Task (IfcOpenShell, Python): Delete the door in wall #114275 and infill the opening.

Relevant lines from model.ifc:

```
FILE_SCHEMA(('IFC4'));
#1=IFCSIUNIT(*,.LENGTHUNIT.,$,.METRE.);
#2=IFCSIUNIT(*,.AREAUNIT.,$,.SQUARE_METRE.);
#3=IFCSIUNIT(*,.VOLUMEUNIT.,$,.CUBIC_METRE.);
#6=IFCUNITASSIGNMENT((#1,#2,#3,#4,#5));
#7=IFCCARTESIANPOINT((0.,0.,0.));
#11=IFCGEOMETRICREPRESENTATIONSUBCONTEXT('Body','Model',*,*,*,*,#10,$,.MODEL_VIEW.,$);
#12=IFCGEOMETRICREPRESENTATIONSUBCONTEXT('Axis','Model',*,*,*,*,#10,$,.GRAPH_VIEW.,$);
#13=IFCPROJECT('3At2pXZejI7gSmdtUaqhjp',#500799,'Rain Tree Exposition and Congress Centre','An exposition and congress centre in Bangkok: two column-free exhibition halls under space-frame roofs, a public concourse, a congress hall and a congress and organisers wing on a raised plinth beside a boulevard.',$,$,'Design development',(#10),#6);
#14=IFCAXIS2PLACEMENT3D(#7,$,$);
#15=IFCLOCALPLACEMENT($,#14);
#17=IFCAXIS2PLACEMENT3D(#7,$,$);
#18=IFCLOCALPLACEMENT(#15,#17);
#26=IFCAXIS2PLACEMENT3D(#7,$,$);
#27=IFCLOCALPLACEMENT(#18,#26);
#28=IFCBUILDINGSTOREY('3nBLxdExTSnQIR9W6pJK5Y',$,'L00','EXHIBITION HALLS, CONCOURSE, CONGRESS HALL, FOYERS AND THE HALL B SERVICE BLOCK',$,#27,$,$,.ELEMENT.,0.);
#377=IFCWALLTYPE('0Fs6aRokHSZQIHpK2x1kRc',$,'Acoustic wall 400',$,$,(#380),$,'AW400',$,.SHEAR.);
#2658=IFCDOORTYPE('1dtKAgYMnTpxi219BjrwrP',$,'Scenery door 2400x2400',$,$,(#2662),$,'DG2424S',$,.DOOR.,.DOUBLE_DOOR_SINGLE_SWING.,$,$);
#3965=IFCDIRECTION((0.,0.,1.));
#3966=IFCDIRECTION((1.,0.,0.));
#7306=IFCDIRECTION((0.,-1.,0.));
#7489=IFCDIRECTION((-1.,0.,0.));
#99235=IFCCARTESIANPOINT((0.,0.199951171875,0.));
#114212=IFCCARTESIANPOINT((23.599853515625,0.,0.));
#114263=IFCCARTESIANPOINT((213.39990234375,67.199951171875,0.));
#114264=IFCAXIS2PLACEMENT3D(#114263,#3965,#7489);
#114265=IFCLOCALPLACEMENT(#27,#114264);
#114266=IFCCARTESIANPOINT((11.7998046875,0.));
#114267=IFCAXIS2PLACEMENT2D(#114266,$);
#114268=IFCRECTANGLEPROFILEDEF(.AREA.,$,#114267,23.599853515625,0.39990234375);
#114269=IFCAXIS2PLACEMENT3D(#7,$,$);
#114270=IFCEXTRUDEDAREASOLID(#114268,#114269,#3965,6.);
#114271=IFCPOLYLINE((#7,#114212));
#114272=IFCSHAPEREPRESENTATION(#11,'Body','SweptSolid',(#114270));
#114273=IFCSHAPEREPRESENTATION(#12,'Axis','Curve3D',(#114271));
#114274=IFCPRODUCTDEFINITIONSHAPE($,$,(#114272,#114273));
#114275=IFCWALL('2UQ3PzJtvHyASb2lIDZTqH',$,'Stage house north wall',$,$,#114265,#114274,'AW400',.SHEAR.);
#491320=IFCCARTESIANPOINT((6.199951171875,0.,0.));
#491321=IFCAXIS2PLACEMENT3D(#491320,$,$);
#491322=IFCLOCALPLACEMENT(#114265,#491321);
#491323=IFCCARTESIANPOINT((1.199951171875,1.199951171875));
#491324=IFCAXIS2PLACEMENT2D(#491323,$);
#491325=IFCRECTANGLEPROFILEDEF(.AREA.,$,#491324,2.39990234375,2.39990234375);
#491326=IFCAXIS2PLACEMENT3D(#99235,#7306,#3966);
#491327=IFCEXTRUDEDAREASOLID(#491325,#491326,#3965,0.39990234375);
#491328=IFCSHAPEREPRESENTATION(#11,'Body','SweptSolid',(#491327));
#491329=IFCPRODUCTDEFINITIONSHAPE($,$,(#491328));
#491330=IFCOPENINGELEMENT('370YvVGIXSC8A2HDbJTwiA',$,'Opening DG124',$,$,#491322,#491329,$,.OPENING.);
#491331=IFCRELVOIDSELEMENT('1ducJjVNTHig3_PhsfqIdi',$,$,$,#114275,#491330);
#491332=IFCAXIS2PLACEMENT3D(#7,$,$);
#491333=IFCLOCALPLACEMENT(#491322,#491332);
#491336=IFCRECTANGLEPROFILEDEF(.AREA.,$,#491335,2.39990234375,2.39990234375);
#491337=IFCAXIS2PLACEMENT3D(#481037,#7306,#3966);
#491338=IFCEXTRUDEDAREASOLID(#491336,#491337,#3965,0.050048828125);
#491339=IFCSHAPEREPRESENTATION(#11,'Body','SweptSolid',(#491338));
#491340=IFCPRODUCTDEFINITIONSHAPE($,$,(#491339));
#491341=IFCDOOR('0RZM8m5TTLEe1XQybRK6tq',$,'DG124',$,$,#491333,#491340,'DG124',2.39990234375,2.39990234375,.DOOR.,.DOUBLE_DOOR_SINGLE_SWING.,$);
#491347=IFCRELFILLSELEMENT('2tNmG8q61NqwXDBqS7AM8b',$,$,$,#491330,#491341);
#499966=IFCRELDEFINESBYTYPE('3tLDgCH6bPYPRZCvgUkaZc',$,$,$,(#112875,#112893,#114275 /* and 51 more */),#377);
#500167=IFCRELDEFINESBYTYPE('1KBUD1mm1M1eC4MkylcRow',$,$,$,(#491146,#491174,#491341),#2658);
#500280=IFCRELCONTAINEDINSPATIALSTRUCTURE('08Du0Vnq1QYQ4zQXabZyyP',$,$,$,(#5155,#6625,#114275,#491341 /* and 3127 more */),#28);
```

```python
import ifcopenshell
import ifcopenshell.api.feature
import ifcopenshell.api.root
import ifcopenshell.geom
import ifcopenshell.util.shape

model = ifcopenshell.open("model.ifc")
settings = ifcopenshell.geom.settings()


def volume(element):
    """Net volume in cubic metres, openings subtracted."""
    shape = ifcopenshell.geom.create_shape(settings, element)
    return ifcopenshell.util.shape.get_volume(shape.geometry)


door = model.by_guid("0RZM8m5TTLEe1XQybRK6tq")
opening = door.FillsVoids[0].RelatingOpeningElement
wall = opening.VoidsElements[0].RelatingBuildingElement
before = volume(wall)

ifcopenshell.api.root.remove_product(model, product=door)
ifcopenshell.api.feature.remove_feature(model, feature=opening)

after = volume(wall)

print(f"wall volume {before:.3f} -> {after:.3f} m3")

model.write("model_edited.ifc")
```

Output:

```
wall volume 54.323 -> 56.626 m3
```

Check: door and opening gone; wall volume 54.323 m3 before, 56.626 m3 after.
